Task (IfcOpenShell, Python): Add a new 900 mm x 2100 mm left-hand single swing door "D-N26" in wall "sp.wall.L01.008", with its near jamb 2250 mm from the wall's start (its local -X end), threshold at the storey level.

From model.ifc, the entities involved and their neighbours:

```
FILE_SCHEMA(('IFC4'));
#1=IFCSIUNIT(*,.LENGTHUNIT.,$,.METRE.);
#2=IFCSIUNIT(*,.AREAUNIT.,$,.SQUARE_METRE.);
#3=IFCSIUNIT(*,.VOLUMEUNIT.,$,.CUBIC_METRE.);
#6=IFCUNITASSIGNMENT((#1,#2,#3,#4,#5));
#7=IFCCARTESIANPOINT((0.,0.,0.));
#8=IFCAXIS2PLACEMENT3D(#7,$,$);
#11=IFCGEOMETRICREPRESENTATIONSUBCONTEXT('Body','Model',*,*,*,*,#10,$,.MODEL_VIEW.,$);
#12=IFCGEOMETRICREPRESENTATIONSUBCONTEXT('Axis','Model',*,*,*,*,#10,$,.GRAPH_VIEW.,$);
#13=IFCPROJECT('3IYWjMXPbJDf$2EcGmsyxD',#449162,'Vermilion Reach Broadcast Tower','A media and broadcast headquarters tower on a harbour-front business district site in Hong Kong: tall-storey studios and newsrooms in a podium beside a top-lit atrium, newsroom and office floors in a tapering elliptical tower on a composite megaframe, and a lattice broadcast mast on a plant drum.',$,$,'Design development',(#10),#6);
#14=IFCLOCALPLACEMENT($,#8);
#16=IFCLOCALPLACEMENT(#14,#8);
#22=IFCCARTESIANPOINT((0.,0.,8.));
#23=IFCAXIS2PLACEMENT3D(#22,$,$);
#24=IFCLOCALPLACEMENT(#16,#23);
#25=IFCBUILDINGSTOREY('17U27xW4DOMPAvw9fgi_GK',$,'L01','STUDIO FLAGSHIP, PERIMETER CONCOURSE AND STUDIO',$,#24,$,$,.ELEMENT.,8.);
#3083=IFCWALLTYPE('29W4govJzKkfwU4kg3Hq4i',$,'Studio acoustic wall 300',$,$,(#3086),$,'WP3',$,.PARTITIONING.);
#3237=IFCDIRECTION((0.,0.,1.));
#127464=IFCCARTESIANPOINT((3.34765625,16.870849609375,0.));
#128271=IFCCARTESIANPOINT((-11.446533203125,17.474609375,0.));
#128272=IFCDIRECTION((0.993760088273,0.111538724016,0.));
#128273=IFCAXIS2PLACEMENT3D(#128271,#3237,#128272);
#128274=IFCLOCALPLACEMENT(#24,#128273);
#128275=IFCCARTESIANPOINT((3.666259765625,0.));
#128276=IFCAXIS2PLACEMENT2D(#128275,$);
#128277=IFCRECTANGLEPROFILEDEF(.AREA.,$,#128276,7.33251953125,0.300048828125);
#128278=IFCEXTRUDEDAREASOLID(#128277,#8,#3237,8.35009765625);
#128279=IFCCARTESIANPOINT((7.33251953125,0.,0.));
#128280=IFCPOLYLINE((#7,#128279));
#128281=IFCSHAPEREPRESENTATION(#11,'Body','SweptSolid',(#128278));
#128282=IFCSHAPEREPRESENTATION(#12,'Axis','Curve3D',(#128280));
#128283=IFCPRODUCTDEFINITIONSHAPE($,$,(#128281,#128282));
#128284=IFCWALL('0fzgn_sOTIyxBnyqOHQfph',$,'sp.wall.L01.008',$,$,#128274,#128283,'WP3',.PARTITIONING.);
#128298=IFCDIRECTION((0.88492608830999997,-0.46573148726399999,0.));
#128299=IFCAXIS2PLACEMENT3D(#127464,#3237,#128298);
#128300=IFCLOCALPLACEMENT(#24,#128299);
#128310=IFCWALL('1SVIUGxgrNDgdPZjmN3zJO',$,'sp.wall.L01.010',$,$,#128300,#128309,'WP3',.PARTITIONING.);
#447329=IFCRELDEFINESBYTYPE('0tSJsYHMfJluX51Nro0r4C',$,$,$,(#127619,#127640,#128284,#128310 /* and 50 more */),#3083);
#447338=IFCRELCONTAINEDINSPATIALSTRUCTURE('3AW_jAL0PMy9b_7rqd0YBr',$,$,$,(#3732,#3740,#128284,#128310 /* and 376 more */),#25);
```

```python
import numpy as np
import ifcopenshell
import ifcopenshell.api.feature
import ifcopenshell.api.geometry
import ifcopenshell.api.root
import ifcopenshell.api.spatial
import ifcopenshell.geom
import ifcopenshell.util.element
import ifcopenshell.util.placement
import ifcopenshell.util.representation
import ifcopenshell.util.shape
import ifcopenshell.util.unit

model = ifcopenshell.open("model.ifc")
unit_scale = ifcopenshell.util.unit.calculate_unit_scale(model)
settings = ifcopenshell.geom.settings()


def volume(element):
    """Net volume in cubic metres, openings subtracted."""
    shape = ifcopenshell.geom.create_shape(settings, element)
    return ifcopenshell.util.shape.get_volume(shape.geometry)


wall = model.by_guid("0fzgn_sOTIyxBnyqOHQfph")
storey = ifcopenshell.util.element.get_container(wall, ifc_class="IfcBuildingStorey")
context = ifcopenshell.util.representation.get_context(model, "Model", "Body", "MODEL_VIEW")
before = volume(wall)

width, height, from_end, sill = 0.9, 2.1, 2.25, 0.0  # metres

# The wall runs along its own X axis, and the end named is its -X end.
wall_shape = ifcopenshell.geom.create_shape(settings, wall)
x, y, z = ifcopenshell.util.shape.get_vertices(wall_shape.geometry).T
start = x.min() + from_end
face, thickness = float(y.min()), float(y.max() - y.min())
wall_matrix = ifcopenshell.util.placement.get_local_placement(wall.ObjectPlacement)
level = ifcopenshell.util.placement.get_local_placement(storey.ObjectPlacement)[2, 3]


def in_wall(x, y):
    """Placement at x, y metres in the wall's axes, at sill height."""
    matrix = wall_matrix.copy()
    matrix[:, 3] = wall_matrix @ np.array([x / unit_scale, y / unit_scale, 0.0, 1.0])
    matrix[2, 3] = level + sill / unit_scale
    return matrix


# Opening: a box that overshoots both wall faces by 50 mm.
opening = ifcopenshell.api.root.create_entity(model, ifc_class="IfcOpeningElement", predefined_type="OPENING")
box = ifcopenshell.api.geometry.add_wall_representation(
    model, context=context, length=width, height=height, thickness=thickness + 0.1
)
ifcopenshell.api.geometry.assign_representation(model, product=opening, representation=box)
ifcopenshell.api.geometry.edit_object_placement(model, product=opening, matrix=in_wall(start, face - 0.05), is_si=False)
ifcopenshell.api.feature.add_feature(model, feature=opening, element=wall)

door = ifcopenshell.api.root.create_entity(model, ifc_class="IfcDoor", name="D-N26", predefined_type="DOOR")
door.OverallWidth, door.OverallHeight = width / unit_scale, height / unit_scale
door.OperationType = "SINGLE_SWING_LEFT"
body = ifcopenshell.api.geometry.add_door_representation(
    model,
    context=context,
    overall_width=door.OverallWidth,
    overall_height=door.OverallHeight,
    operation_type="SINGLE_SWING_LEFT",
    lining_properties={"LiningDepth": thickness / unit_scale, "ThresholdDepth": thickness / unit_scale},
)
ifcopenshell.api.geometry.assign_representation(model, product=door, representation=body)
ifcopenshell.api.spatial.assign_container(model, products=[door], relating_structure=storey)
ifcopenshell.api.feature.add_filling(model, opening=opening, element=door)

# The lining spans the wall, so the door starts at the wall face.
ifcopenshell.api.geometry.edit_object_placement(model, product=door, matrix=in_wall(start, face), is_si=False)

after = volume(wall)

print(f"wall volume {before:.3f} -> {after:.3f} m3")

model.write("model_v2.ifc")
```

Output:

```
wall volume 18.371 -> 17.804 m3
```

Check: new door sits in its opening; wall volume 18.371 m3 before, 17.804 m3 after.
